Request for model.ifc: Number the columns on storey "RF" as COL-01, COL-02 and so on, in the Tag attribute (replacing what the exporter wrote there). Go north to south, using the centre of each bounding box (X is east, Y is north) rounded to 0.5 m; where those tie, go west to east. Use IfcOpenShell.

First a look at what the model holds.

```python
import ifcopenshell
import ifcopenshell.util.element
import ifcopenshell.util.placement

model = ifcopenshell.open("model.ifc")
print(model.schema)
storey = next(s for s in model.by_type("IfcBuildingStorey") if s.Name == "RF")
columns = [e for e in ifcopenshell.util.element.get_decomposition(storey) if e.is_a("IfcColumn")]
for e in sorted(columns, key=lambda e: e.id()):
    origin = ifcopenshell.util.placement.get_local_placement(e.ObjectPlacement)[:3, 3]
    print(e.id(), e.Tag, e.Name, origin.round(2) + 0.0, sep=" | ")
```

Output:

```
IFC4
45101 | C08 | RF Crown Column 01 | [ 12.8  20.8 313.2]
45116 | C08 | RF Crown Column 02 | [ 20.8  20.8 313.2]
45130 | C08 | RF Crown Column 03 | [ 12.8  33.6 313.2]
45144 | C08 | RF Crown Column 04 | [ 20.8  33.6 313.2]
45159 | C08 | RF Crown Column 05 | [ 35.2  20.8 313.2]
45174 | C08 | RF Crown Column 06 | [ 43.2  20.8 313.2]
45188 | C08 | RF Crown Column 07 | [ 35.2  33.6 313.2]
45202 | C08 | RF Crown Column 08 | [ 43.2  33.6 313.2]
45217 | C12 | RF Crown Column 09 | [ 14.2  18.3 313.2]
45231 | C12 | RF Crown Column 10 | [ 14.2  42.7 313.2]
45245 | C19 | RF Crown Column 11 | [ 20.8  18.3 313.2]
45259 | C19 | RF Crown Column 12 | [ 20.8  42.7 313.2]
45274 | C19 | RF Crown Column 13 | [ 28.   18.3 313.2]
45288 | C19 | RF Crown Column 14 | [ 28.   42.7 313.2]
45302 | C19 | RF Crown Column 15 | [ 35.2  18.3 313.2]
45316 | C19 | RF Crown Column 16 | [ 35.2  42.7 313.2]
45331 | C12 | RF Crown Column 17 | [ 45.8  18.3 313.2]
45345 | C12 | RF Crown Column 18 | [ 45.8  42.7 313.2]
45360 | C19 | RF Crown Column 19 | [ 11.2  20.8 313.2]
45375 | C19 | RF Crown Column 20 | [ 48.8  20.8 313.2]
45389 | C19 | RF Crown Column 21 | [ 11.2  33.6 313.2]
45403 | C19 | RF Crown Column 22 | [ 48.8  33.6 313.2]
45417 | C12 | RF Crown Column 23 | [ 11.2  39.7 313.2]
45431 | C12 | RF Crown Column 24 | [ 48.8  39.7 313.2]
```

```python
import ifcopenshell
import ifcopenshell.geom
import ifcopenshell.util.element
import ifcopenshell.util.shape

model = ifcopenshell.open("model.ifc")
settings = ifcopenshell.geom.settings()
settings.set("use-world-coords", True)


def centre(element):
    shape = ifcopenshell.geom.create_shape(settings, element)
    return ifcopenshell.util.shape.get_bbox_centroid(shape.geometry)


storey = next(s for s in model.by_type("IfcBuildingStorey") if s.Name == "RF")
columns = [e for e in ifcopenshell.util.element.get_decomposition(storey) if e.is_a("IfcColumn")]

# Insertion points can sit at a corner or the storey origin, so sort by the geometry (in metres).
centres = {e: centre(e) for e in columns}
columns.sort(key=lambda e: (-round(centres[e][1] / 0.5), centres[e][0]))

for i, e in enumerate(columns, start=1):
    number = f"COL-{i:02d}"
    e.Tag = number
    print(e.id(), number)

model.write("model_v2.ifc")
```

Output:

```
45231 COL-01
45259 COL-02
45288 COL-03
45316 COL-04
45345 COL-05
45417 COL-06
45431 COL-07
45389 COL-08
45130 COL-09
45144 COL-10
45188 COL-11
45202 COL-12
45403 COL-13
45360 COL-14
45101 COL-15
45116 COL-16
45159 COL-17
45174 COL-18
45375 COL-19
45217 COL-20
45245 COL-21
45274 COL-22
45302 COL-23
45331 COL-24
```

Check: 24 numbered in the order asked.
